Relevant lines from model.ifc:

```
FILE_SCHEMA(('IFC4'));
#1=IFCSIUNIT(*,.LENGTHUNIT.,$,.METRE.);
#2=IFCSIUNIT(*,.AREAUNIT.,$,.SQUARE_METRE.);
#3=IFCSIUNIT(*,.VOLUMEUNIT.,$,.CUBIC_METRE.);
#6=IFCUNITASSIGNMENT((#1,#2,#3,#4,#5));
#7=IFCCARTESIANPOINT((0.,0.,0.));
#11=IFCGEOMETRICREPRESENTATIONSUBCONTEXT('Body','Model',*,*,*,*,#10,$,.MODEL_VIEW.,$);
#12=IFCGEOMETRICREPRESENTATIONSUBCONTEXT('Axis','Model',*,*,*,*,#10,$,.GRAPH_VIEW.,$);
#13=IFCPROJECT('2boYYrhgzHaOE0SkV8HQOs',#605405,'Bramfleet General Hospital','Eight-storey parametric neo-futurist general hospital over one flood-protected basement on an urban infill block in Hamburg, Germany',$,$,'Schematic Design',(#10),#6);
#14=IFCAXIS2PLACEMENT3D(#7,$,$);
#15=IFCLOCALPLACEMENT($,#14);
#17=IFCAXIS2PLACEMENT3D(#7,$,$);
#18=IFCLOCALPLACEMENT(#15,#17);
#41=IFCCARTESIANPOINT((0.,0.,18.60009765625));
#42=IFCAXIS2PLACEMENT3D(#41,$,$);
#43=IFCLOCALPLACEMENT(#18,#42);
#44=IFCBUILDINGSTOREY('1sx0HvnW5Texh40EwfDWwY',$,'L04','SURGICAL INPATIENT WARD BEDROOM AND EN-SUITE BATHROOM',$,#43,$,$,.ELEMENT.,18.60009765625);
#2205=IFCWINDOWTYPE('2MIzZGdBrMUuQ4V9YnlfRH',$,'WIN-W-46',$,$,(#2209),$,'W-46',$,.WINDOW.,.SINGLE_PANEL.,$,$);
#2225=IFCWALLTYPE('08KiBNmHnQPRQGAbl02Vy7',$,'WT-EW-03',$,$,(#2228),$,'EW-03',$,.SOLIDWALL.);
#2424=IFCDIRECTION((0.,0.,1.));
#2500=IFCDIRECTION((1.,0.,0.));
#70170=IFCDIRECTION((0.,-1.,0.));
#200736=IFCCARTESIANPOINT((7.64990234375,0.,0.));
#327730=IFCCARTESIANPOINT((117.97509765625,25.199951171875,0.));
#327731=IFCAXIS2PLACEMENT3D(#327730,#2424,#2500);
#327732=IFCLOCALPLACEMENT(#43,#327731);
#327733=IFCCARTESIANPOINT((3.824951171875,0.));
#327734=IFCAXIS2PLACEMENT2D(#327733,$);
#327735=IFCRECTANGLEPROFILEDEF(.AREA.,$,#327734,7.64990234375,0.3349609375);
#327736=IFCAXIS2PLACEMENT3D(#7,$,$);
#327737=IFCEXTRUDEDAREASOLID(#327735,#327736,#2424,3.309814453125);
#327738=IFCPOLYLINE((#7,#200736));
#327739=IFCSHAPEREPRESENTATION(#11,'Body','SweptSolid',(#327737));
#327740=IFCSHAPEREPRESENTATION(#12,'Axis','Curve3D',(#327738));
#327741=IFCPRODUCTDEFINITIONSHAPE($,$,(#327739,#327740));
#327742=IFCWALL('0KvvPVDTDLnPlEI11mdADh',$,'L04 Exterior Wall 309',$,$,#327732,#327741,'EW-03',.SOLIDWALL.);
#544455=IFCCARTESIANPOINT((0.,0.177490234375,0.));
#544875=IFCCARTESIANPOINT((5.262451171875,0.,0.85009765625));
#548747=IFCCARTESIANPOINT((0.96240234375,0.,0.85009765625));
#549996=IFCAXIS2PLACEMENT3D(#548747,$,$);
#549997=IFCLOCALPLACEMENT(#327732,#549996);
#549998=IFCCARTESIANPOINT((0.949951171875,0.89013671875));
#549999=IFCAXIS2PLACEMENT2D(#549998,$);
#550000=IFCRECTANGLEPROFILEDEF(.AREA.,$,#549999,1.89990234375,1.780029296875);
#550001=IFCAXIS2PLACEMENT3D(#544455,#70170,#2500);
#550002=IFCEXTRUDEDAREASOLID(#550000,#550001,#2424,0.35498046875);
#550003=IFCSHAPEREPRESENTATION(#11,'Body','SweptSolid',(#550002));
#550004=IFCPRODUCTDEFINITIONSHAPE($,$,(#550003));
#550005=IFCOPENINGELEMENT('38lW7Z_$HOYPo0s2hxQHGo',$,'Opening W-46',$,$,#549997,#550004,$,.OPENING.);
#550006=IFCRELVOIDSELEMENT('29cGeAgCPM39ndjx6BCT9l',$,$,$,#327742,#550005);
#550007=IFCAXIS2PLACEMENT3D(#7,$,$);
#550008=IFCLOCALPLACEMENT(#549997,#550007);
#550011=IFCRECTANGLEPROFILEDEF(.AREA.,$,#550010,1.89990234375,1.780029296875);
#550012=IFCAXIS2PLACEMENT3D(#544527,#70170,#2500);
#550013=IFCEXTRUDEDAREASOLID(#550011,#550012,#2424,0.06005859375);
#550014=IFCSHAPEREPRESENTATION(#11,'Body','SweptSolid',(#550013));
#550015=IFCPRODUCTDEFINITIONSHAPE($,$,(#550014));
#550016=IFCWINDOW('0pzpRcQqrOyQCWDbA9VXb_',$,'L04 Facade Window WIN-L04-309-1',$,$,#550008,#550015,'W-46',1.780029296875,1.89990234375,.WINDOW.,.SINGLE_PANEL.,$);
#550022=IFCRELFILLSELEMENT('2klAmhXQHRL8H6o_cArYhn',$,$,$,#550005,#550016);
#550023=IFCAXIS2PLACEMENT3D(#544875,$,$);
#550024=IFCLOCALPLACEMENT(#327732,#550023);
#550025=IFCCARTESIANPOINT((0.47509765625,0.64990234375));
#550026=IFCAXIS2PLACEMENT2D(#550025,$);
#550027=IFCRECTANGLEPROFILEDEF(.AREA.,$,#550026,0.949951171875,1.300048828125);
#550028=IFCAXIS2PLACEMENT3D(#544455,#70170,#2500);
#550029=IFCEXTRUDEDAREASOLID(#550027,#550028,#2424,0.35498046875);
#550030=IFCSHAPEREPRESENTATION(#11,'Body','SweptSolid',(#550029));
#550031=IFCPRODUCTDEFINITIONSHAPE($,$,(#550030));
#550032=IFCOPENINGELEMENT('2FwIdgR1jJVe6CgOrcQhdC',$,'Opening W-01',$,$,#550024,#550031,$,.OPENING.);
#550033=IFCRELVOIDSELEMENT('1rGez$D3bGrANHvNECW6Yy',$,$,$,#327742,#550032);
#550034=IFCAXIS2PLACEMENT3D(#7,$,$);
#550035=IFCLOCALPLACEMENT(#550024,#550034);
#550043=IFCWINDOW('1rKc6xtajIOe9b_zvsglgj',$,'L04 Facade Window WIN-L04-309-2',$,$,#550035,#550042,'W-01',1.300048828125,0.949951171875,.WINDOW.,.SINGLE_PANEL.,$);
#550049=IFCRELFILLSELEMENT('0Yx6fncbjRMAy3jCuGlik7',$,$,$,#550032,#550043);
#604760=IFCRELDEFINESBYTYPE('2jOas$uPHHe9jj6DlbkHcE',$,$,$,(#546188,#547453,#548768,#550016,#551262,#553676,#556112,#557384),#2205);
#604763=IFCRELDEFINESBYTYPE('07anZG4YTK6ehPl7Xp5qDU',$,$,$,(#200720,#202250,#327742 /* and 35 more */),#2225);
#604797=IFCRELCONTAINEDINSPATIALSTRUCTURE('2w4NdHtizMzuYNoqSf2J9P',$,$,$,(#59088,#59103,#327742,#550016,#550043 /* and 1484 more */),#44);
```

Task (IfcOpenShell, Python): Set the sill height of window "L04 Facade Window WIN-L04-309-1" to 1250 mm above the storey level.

```python
import numpy as np
import ifcopenshell
import ifcopenshell.api.geometry
import ifcopenshell.geom
import ifcopenshell.util.element
import ifcopenshell.util.placement
import ifcopenshell.util.shape
import ifcopenshell.util.unit

model = ifcopenshell.open("model.ifc")
unit_scale = ifcopenshell.util.unit.calculate_unit_scale(model)

window = model.by_guid("0pzpRcQqrOyQCWDbA9VXb_")
opening = window.FillsVoids[0].RelatingOpeningElement
storey = ifcopenshell.util.element.get_container(window, ifc_class="IfcBuildingStorey")
level = ifcopenshell.util.placement.get_local_placement(storey.ObjectPlacement)[2, 3]

# The opening's origin need not be at the sill, so measure its lowest point.
shape = ifcopenshell.geom.create_shape(ifcopenshell.geom.settings(), opening)
bottom = ifcopenshell.util.shape.get_shape_bottom_elevation(shape, shape.geometry) / unit_scale
dz = level + 1.25 - bottom

shift = np.array([0.0, 0.0, dz])
# The window is placed relative to its opening, so it follows when the opening moves.
matrix = ifcopenshell.util.placement.get_local_placement(opening.ObjectPlacement)
matrix[:3, 3] += shift
ifcopenshell.api.geometry.edit_object_placement(
    model, product=opening, matrix=matrix, is_si=False, should_transform_children=True
)

print(f"moved by {dz * unit_scale:+.3f} m")

model.write("model_edited.ifc")
```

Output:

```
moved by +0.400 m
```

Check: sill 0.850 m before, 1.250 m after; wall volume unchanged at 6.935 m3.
